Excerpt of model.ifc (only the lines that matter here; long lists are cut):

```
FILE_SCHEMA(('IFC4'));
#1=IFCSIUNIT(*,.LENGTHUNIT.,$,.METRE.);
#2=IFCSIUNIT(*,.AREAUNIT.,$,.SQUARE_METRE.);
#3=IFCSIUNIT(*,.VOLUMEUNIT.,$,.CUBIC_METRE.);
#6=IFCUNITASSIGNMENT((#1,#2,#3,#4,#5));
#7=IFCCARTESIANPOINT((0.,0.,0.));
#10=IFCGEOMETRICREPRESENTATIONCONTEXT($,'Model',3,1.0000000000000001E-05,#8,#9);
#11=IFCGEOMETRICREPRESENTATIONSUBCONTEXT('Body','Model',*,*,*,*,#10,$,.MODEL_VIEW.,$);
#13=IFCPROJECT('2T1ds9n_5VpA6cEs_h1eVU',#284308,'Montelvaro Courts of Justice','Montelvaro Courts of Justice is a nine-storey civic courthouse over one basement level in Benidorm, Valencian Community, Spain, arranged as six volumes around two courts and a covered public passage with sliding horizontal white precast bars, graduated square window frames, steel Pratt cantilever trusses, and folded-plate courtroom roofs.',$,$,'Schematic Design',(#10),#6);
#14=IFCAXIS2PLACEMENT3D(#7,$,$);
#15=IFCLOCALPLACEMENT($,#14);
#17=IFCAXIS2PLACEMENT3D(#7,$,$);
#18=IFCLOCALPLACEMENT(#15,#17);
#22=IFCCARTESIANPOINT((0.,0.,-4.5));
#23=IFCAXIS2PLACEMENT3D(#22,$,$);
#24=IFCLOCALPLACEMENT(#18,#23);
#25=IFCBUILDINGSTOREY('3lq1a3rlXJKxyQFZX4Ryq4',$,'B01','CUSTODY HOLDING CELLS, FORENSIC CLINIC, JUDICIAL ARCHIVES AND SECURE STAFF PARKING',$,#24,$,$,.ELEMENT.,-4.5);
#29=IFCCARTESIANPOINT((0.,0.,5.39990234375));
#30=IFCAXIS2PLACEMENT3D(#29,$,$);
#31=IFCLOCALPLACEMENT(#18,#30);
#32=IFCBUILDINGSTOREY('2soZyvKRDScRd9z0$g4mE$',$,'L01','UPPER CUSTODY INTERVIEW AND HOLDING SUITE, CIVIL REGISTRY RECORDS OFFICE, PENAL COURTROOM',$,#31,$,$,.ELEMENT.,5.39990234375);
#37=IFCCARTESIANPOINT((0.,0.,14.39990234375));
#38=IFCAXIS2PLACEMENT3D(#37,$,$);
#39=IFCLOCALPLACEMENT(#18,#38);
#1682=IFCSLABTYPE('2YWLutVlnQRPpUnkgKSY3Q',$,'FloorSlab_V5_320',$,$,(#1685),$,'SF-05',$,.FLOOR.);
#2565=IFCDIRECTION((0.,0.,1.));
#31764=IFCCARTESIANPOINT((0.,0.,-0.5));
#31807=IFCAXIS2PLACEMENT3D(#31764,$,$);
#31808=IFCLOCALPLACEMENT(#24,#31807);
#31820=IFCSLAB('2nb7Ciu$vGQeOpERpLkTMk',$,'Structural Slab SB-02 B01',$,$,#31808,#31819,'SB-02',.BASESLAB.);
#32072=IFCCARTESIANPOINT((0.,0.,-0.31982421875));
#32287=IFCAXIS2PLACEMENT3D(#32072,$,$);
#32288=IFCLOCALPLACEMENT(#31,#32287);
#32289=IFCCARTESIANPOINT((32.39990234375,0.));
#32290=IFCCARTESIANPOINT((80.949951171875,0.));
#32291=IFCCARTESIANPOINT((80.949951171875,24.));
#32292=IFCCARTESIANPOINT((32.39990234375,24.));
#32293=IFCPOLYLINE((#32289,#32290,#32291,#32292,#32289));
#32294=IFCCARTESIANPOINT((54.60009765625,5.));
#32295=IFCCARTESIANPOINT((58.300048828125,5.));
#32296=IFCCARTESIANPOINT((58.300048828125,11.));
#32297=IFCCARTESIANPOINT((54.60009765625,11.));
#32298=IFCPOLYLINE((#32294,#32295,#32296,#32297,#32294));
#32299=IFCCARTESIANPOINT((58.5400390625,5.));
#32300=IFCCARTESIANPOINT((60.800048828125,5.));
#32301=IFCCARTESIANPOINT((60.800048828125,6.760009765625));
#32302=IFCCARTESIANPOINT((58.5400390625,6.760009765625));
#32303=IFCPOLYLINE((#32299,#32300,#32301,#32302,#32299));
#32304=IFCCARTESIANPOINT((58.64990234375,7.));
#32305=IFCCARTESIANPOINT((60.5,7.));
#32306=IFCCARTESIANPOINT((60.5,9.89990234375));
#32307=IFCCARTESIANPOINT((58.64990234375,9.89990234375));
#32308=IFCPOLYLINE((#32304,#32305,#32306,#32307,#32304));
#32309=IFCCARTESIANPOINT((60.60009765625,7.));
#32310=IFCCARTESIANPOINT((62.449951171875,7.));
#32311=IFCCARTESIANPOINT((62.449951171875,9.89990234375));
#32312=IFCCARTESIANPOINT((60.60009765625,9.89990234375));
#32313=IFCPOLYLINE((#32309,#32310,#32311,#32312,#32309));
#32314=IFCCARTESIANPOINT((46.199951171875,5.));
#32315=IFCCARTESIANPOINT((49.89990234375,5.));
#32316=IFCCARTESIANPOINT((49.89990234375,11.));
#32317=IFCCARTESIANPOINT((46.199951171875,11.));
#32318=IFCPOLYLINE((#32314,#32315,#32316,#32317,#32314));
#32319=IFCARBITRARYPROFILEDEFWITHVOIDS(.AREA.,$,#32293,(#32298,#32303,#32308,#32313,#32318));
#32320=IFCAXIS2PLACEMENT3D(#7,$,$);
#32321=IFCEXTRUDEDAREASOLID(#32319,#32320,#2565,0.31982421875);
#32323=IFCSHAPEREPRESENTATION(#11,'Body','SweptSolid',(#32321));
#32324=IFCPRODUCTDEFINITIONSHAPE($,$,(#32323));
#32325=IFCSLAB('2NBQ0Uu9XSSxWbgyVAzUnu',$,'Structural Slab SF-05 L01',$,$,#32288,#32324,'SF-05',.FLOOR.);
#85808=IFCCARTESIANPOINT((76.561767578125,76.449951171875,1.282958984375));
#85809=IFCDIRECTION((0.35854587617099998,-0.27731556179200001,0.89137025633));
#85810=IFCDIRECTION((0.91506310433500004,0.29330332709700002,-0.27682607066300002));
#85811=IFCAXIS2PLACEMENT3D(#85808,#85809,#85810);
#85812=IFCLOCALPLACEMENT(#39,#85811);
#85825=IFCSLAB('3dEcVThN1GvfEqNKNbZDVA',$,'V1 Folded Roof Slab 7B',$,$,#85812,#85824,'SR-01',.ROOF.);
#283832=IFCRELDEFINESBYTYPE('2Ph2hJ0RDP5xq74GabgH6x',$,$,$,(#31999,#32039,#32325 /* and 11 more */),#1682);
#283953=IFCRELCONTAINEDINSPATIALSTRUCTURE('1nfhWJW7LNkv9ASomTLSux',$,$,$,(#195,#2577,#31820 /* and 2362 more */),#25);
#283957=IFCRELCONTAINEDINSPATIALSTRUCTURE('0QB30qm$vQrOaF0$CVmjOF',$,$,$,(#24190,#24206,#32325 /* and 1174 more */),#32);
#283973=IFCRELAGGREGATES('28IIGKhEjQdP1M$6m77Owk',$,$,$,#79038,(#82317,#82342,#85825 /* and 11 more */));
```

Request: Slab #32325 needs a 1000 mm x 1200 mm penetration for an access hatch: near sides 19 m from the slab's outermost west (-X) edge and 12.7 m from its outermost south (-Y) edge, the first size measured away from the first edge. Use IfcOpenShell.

```python
import numpy as np
import ifcopenshell
import ifcopenshell.api.feature
import ifcopenshell.api.geometry
import ifcopenshell.api.root
import ifcopenshell.geom
import ifcopenshell.util.placement
import ifcopenshell.util.representation
import ifcopenshell.util.shape
import ifcopenshell.util.unit

model = ifcopenshell.open("model.ifc")
unit_scale = ifcopenshell.util.unit.calculate_unit_scale(model)
settings = ifcopenshell.geom.settings()


def volume(element):
    """Net volume in cubic metres, openings subtracted."""
    shape = ifcopenshell.geom.create_shape(settings, element)
    return ifcopenshell.util.shape.get_volume(shape.geometry)


slab = model.by_id(32325)
before = volume(slab)

# Extent in the slab's own axes, in metres. The edges named are its -X and -Y sides.
slab_shape = ifcopenshell.geom.create_shape(settings, slab)
vertices = ifcopenshell.util.shape.get_vertices(slab_shape.geometry)
x_min, y_min, bottom = vertices.min(axis=0)
top = vertices[:, 2].max()

opening = ifcopenshell.api.root.create_entity(model, ifc_class="IfcOpeningElement", name="Access hatch opening", predefined_type="OPENING")
context = ifcopenshell.util.representation.get_context(model, "Model", "Body", "MODEL_VIEW")
width, depth = 1, 1.2
outline = [(0.0, 0.0), (width, 0.0), (width, depth), (0.0, depth), (0.0, 0.0)]
# Overshoot both faces by 50 mm so the cut is clean.
shape = ifcopenshell.api.geometry.add_slab_representation(
    model, context=context, depth=top - bottom + 0.1, polyline=outline
)
ifcopenshell.api.geometry.assign_representation(model, product=opening, representation=shape)

matrix = ifcopenshell.util.placement.get_local_placement(slab.ObjectPlacement)
matrix[:, 3] = matrix @ np.append(np.array([x_min + 19, y_min + 12.7, bottom - 0.05]) / unit_scale, 1.0)
ifcopenshell.api.geometry.edit_object_placement(model, product=opening, matrix=matrix, is_si=False)
ifcopenshell.api.feature.add_feature(model, feature=opening, element=slab)

after = volume(slab)

print(f"slab volume {before:.3f} -> {after:.3f} m3")

model.write("model_v2.ifc")
```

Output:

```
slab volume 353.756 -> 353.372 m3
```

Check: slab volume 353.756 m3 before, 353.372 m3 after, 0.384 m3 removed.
